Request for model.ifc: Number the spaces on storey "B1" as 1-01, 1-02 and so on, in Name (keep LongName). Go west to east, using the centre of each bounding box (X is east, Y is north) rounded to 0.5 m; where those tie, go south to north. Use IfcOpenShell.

First a look at what the model holds.

```python
import ifcopenshell
import ifcopenshell.util.element
import ifcopenshell.util.placement

model = ifcopenshell.open("model.ifc")
print(model.schema)
storey = next(s for s in model.by_type("IfcBuildingStorey") if s.Name == "B1")
spaces = [e for e in ifcopenshell.util.element.get_decomposition(storey) if e.is_a("IfcSpace")]
for e in sorted(spaces, key=lambda e: e.id()):
    origin = ifcopenshell.util.placement.get_local_placement(e.ObjectPlacement)[:3, 3]
    print(e.id(), e.Name, e.LongName, origin.round(2) + 0.0, sep=" | ")
```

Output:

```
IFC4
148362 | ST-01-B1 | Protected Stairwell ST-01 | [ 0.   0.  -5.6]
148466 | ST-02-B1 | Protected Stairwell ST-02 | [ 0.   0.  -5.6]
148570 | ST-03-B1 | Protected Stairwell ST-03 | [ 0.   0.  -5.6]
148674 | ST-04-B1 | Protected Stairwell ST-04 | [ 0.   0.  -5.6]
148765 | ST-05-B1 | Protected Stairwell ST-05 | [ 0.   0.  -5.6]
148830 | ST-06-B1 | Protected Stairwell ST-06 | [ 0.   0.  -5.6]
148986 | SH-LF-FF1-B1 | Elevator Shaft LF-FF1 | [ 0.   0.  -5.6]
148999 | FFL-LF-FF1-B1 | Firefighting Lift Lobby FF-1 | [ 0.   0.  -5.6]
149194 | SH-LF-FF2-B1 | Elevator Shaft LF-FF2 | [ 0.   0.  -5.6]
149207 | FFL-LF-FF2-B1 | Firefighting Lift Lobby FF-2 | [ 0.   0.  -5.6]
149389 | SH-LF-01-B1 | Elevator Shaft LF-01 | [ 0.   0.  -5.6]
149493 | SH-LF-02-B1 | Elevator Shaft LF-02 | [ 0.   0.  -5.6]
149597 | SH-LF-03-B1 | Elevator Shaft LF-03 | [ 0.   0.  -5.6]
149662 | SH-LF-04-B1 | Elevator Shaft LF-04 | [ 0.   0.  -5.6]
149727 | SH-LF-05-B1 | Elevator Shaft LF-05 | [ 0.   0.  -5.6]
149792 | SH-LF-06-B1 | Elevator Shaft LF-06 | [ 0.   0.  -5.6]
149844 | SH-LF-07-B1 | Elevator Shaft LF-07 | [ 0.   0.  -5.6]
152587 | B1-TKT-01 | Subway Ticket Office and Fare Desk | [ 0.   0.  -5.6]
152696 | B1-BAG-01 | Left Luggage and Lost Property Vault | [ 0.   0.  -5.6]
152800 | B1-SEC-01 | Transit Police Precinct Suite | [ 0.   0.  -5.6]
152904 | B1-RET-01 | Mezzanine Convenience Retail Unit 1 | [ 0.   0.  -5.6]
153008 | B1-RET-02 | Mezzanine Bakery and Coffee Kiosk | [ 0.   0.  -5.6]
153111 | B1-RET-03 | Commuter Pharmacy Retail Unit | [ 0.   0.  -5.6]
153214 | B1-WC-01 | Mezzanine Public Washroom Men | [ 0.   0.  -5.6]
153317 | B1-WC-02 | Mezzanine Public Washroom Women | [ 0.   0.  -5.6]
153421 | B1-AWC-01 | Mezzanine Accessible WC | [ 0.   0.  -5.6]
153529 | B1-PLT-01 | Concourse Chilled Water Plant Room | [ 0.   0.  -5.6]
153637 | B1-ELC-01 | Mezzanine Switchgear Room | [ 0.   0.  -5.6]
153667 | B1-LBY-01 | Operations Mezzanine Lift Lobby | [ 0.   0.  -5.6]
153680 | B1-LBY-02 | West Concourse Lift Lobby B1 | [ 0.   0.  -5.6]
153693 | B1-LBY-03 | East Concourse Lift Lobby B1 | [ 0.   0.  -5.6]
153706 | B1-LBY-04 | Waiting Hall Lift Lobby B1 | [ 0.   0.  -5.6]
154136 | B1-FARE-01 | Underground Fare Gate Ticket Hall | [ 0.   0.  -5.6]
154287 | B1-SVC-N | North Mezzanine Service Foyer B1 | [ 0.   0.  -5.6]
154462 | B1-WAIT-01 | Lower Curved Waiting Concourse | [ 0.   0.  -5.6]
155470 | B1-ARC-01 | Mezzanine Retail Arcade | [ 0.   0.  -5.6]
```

```python
import ifcopenshell
import ifcopenshell.geom
import ifcopenshell.util.element
import ifcopenshell.util.shape

model = ifcopenshell.open("model.ifc")
settings = ifcopenshell.geom.settings()
settings.set("use-world-coords", True)


def centre(element):
    shape = ifcopenshell.geom.create_shape(settings, element)
    return ifcopenshell.util.shape.get_bbox_centroid(shape.geometry)


storey = next(s for s in model.by_type("IfcBuildingStorey") if s.Name == "B1")
spaces = [e for e in ifcopenshell.util.element.get_decomposition(storey) if e.is_a("IfcSpace")]

# Insertion points can sit at a corner or the storey origin, so sort by the geometry (in metres).
centres = {e: centre(e) for e in spaces}
spaces.sort(key=lambda e: (round(centres[e][0] / 0.5), centres[e][1]))

for i, e in enumerate(spaces, start=1):
    number = f"1-{i:02d}"
    e.Name = number
    print(e.id(), number)

model.write("model_rev.ifc")
```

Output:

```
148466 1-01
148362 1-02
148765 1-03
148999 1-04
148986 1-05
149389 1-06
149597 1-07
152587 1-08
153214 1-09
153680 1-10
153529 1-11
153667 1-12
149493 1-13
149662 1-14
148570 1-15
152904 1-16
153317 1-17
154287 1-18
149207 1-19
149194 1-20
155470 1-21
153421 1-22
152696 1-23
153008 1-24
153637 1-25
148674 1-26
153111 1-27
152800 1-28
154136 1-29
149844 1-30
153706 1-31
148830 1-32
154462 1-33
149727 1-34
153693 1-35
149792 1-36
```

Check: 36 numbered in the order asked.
